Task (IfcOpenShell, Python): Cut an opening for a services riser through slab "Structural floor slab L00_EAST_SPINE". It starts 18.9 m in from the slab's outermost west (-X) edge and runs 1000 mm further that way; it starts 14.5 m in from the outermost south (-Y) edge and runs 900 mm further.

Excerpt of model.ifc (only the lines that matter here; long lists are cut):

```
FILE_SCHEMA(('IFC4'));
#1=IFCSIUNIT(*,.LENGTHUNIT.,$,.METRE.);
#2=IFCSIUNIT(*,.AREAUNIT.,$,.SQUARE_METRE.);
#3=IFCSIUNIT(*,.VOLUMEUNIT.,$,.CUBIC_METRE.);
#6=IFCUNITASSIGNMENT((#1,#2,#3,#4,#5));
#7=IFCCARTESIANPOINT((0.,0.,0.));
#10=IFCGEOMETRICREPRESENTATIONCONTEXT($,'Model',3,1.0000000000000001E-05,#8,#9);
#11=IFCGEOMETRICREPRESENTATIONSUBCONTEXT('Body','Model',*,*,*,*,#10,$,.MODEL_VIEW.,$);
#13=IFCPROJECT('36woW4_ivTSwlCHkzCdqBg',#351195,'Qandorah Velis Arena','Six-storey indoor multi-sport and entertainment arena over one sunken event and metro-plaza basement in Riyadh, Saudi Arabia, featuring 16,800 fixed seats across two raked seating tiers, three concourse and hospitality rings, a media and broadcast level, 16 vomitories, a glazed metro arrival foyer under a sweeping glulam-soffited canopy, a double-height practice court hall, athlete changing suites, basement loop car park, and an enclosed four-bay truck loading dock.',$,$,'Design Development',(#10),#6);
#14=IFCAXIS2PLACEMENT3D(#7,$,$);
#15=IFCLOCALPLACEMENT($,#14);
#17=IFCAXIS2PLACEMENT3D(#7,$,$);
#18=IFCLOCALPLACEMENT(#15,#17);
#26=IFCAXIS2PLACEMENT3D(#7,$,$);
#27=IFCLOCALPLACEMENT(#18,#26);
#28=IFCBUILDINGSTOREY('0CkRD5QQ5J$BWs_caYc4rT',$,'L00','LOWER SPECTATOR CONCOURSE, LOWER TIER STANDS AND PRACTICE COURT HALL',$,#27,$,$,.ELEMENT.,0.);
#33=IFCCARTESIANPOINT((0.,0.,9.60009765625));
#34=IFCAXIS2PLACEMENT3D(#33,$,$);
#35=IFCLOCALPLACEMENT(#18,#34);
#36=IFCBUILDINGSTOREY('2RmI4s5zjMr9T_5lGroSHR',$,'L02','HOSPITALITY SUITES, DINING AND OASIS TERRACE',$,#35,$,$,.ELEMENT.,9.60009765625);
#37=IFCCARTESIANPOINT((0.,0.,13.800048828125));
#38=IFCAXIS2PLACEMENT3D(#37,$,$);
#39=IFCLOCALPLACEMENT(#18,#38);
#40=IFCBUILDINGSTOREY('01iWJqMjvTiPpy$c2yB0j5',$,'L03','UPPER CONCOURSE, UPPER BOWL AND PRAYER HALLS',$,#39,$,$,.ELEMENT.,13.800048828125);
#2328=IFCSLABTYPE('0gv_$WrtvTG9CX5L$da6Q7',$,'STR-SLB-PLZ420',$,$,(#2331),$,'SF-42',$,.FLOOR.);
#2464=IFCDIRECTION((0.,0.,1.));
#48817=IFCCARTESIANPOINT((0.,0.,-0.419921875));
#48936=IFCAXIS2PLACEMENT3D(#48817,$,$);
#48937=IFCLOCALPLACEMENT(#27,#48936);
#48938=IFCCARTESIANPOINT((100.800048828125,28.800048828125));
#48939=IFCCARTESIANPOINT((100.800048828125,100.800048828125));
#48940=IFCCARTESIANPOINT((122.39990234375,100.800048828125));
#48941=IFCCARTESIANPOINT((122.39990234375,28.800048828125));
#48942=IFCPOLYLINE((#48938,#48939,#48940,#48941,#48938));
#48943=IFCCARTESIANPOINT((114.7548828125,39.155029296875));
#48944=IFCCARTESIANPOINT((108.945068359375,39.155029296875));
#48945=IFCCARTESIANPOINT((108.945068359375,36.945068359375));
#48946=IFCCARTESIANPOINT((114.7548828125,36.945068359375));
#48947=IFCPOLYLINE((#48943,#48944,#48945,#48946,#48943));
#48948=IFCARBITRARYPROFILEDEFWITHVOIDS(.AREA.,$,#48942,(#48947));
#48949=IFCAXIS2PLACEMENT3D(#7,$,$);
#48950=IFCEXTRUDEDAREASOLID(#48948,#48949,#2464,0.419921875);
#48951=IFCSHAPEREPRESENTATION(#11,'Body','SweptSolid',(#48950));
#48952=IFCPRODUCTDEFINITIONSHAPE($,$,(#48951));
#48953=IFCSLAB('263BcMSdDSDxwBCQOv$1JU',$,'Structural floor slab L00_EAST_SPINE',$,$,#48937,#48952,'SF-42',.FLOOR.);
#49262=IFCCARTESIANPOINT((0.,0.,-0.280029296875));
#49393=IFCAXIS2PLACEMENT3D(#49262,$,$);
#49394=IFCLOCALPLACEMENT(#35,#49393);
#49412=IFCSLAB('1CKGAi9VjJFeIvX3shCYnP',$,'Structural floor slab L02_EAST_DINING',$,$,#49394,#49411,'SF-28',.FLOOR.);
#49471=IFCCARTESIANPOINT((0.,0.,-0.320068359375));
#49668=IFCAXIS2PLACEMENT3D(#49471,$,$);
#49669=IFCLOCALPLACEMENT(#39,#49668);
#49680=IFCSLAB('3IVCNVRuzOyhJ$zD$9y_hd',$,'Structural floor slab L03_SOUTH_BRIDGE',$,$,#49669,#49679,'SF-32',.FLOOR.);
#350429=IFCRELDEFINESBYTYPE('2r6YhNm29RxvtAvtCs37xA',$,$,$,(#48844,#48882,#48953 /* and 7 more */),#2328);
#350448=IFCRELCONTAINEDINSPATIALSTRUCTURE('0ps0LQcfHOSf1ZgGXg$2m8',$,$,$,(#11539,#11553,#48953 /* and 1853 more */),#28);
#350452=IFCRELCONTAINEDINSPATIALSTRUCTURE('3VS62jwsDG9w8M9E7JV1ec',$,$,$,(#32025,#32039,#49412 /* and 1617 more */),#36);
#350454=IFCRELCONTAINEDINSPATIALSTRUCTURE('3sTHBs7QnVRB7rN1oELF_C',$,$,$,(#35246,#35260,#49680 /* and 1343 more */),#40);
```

```python
import numpy as np
import ifcopenshell
import ifcopenshell.api.feature
import ifcopenshell.api.geometry
import ifcopenshell.api.root
import ifcopenshell.geom
import ifcopenshell.util.placement
import ifcopenshell.util.representation
import ifcopenshell.util.shape
import ifcopenshell.util.unit

model = ifcopenshell.open("model.ifc")
unit_scale = ifcopenshell.util.unit.calculate_unit_scale(model)
settings = ifcopenshell.geom.settings()


def volume(element):
    """Net volume in cubic metres, openings subtracted."""
    shape = ifcopenshell.geom.create_shape(settings, element)
    return ifcopenshell.util.shape.get_volume(shape.geometry)


slab = model.by_guid("263BcMSdDSDxwBCQOv$1JU")
before = volume(slab)

# Extent in the slab's own axes, in metres. The edges named are its -X and -Y sides.
slab_shape = ifcopenshell.geom.create_shape(settings, slab)
vertices = ifcopenshell.util.shape.get_vertices(slab_shape.geometry)
x_min, y_min, bottom = vertices.min(axis=0)
top = vertices[:, 2].max()

opening = ifcopenshell.api.root.create_entity(model, ifc_class="IfcOpeningElement", name="Services riser opening", predefined_type="OPENING")
context = ifcopenshell.util.representation.get_context(model, "Model", "Body", "MODEL_VIEW")
width, depth = 1, 0.9
outline = [(0.0, 0.0), (width, 0.0), (width, depth), (0.0, depth), (0.0, 0.0)]
# Overshoot both faces by 50 mm so the cut is clean.
shape = ifcopenshell.api.geometry.add_slab_representation(
    model, context=context, depth=top - bottom + 0.1, polyline=outline
)
ifcopenshell.api.geometry.assign_representation(model, product=opening, representation=shape)

matrix = ifcopenshell.util.placement.get_local_placement(slab.ObjectPlacement)
matrix[:, 3] = matrix @ np.append(np.array([x_min + 18.9, y_min + 14.5, bottom - 0.05]) / unit_scale, 1.0)
ifcopenshell.api.geometry.edit_object_placement(model, product=opening, matrix=matrix, is_si=False)
ifcopenshell.api.feature.add_feature(model, feature=opening, element=slab)

after = volume(slab)

print(f"slab volume {before:.3f} -> {after:.3f} m3")

model.write("model_edited.ifc")
```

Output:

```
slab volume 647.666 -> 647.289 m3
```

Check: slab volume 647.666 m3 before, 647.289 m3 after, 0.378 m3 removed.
